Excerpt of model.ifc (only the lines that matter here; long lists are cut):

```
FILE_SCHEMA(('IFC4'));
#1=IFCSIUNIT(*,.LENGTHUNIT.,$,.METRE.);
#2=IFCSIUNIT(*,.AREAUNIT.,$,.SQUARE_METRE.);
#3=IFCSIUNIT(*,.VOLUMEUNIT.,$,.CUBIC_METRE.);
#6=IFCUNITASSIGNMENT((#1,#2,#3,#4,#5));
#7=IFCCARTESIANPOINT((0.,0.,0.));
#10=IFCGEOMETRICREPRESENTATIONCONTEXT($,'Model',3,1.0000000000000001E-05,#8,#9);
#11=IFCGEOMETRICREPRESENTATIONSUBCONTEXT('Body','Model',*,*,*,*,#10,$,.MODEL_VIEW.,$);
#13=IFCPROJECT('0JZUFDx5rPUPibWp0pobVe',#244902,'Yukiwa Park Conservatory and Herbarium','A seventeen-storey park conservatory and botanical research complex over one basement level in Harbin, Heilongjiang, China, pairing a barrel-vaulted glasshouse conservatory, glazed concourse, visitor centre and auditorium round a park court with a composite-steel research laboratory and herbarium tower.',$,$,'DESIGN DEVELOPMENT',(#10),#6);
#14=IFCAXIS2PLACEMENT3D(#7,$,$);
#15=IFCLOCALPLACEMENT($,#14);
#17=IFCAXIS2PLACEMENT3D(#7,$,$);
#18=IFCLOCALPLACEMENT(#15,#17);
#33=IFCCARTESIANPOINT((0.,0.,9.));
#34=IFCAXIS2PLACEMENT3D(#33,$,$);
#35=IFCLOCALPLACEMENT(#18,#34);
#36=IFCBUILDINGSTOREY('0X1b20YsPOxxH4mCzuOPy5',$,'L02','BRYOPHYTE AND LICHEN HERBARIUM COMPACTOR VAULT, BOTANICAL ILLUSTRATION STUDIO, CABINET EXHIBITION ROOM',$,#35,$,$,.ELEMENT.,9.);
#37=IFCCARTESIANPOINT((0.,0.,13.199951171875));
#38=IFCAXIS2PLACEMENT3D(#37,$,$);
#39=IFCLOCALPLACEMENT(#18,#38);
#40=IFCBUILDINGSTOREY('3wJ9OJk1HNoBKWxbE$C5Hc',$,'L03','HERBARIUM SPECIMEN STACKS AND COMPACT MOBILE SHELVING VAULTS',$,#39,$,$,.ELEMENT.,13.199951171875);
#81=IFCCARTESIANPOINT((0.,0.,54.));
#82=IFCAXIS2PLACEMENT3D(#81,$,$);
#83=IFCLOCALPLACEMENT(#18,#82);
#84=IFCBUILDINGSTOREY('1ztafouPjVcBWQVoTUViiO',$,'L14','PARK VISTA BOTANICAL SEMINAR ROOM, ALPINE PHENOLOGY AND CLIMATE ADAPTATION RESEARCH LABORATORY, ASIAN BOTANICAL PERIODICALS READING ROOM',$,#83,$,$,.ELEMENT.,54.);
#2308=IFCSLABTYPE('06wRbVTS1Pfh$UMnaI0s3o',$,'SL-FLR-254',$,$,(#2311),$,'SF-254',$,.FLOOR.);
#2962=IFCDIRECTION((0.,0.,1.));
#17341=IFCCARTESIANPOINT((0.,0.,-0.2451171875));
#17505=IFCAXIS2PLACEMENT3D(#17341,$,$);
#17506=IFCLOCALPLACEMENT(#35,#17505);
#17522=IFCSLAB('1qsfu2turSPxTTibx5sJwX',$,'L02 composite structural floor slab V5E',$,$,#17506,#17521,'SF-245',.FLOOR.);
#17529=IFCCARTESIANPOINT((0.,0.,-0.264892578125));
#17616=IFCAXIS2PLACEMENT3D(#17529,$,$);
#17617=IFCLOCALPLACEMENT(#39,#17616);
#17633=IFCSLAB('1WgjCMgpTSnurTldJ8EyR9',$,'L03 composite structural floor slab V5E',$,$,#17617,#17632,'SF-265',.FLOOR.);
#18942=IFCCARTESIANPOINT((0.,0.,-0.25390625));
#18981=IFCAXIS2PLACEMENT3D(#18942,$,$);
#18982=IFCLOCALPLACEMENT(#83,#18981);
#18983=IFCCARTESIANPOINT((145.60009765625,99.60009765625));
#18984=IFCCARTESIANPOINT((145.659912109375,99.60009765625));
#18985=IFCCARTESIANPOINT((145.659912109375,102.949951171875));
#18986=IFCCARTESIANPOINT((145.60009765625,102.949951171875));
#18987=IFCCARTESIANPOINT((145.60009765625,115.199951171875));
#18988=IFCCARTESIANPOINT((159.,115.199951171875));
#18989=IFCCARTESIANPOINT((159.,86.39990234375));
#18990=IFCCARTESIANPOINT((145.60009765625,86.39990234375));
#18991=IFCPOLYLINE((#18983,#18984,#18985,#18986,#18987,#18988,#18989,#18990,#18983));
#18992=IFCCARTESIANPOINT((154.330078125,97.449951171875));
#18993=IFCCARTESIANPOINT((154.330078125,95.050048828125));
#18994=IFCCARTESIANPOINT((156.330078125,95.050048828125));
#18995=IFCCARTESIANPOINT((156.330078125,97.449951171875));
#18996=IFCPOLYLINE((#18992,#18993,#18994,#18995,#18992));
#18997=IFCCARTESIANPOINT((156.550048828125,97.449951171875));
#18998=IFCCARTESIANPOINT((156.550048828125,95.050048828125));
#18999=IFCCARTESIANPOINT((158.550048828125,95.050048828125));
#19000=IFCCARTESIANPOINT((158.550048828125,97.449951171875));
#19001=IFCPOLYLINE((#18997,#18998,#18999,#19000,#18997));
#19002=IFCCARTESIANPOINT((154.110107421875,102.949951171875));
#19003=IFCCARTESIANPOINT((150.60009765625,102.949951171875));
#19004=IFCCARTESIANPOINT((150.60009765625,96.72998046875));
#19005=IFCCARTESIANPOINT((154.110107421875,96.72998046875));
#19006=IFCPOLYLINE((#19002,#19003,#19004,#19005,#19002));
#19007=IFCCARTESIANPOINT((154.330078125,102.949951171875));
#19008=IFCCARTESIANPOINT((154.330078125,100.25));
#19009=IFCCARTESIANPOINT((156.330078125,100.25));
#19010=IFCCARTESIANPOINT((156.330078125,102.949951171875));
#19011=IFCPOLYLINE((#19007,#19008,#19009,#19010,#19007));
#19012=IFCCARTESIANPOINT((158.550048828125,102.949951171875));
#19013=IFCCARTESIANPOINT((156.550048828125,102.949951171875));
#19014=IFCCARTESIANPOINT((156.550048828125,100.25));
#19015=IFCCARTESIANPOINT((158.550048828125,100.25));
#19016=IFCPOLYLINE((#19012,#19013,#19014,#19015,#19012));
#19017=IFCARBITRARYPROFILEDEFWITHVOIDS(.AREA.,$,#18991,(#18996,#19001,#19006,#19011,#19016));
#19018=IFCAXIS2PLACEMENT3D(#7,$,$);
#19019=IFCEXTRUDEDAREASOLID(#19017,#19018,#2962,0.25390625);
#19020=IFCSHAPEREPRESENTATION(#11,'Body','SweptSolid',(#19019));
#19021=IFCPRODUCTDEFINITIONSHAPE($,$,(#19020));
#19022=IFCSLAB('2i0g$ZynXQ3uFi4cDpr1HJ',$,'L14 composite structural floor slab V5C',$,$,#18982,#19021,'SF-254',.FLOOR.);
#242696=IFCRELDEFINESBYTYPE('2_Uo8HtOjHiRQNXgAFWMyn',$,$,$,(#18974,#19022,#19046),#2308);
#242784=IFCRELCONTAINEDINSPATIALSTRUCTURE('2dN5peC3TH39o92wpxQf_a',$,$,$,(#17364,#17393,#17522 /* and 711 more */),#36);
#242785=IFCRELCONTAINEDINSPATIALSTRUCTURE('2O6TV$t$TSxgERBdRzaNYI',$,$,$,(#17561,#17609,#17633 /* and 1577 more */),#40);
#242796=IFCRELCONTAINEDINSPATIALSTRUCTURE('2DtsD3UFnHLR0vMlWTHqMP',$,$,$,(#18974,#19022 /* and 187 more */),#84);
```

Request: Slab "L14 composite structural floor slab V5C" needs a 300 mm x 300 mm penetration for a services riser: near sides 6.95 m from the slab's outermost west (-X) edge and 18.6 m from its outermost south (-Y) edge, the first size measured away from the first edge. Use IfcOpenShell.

```python
import numpy as np
import ifcopenshell
import ifcopenshell.api.feature
import ifcopenshell.api.geometry
import ifcopenshell.api.root
import ifcopenshell.geom
import ifcopenshell.util.placement
import ifcopenshell.util.representation
import ifcopenshell.util.shape
import ifcopenshell.util.unit

model = ifcopenshell.open("model.ifc")
unit_scale = ifcopenshell.util.unit.calculate_unit_scale(model)
settings = ifcopenshell.geom.settings()


def volume(element):
    """Net volume in cubic metres, openings subtracted."""
    shape = ifcopenshell.geom.create_shape(settings, element)
    return ifcopenshell.util.shape.get_volume(shape.geometry)


slab = model.by_id(19022)
before = volume(slab)

# Extent in the slab's own axes, in metres. The edges named are its -X and -Y sides.
slab_shape = ifcopenshell.geom.create_shape(settings, slab)
vertices = ifcopenshell.util.shape.get_vertices(slab_shape.geometry)
x_min, y_min, bottom = vertices.min(axis=0)
top = vertices[:, 2].max()

opening = ifcopenshell.api.root.create_entity(model, ifc_class="IfcOpeningElement", name="Services riser opening", predefined_type="OPENING")
context = ifcopenshell.util.representation.get_context(model, "Model", "Body", "MODEL_VIEW")
width, depth = 0.3, 0.3
outline = [(0.0, 0.0), (width, 0.0), (width, depth), (0.0, depth), (0.0, 0.0)]
# Overshoot both faces by 50 mm so the cut is clean.
shape = ifcopenshell.api.geometry.add_slab_representation(
    model, context=context, depth=top - bottom + 0.1, polyline=outline
)
ifcopenshell.api.geometry.assign_representation(model, product=opening, representation=shape)

matrix = ifcopenshell.util.placement.get_local_placement(slab.ObjectPlacement)
matrix[:, 3] = matrix @ np.append(np.array([x_min + 6.95, y_min + 18.6, bottom - 0.05]) / unit_scale, 1.0)
ifcopenshell.api.geometry.edit_object_placement(model, product=opening, matrix=matrix, is_si=False)
ifcopenshell.api.feature.add_feature(model, feature=opening, element=slab)

after = volume(slab)

print(f"slab volume {before:.3f} -> {after:.3f} m3")

model.write("model_rev.ifc")
```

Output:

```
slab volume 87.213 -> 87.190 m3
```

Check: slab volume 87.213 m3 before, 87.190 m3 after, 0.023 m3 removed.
